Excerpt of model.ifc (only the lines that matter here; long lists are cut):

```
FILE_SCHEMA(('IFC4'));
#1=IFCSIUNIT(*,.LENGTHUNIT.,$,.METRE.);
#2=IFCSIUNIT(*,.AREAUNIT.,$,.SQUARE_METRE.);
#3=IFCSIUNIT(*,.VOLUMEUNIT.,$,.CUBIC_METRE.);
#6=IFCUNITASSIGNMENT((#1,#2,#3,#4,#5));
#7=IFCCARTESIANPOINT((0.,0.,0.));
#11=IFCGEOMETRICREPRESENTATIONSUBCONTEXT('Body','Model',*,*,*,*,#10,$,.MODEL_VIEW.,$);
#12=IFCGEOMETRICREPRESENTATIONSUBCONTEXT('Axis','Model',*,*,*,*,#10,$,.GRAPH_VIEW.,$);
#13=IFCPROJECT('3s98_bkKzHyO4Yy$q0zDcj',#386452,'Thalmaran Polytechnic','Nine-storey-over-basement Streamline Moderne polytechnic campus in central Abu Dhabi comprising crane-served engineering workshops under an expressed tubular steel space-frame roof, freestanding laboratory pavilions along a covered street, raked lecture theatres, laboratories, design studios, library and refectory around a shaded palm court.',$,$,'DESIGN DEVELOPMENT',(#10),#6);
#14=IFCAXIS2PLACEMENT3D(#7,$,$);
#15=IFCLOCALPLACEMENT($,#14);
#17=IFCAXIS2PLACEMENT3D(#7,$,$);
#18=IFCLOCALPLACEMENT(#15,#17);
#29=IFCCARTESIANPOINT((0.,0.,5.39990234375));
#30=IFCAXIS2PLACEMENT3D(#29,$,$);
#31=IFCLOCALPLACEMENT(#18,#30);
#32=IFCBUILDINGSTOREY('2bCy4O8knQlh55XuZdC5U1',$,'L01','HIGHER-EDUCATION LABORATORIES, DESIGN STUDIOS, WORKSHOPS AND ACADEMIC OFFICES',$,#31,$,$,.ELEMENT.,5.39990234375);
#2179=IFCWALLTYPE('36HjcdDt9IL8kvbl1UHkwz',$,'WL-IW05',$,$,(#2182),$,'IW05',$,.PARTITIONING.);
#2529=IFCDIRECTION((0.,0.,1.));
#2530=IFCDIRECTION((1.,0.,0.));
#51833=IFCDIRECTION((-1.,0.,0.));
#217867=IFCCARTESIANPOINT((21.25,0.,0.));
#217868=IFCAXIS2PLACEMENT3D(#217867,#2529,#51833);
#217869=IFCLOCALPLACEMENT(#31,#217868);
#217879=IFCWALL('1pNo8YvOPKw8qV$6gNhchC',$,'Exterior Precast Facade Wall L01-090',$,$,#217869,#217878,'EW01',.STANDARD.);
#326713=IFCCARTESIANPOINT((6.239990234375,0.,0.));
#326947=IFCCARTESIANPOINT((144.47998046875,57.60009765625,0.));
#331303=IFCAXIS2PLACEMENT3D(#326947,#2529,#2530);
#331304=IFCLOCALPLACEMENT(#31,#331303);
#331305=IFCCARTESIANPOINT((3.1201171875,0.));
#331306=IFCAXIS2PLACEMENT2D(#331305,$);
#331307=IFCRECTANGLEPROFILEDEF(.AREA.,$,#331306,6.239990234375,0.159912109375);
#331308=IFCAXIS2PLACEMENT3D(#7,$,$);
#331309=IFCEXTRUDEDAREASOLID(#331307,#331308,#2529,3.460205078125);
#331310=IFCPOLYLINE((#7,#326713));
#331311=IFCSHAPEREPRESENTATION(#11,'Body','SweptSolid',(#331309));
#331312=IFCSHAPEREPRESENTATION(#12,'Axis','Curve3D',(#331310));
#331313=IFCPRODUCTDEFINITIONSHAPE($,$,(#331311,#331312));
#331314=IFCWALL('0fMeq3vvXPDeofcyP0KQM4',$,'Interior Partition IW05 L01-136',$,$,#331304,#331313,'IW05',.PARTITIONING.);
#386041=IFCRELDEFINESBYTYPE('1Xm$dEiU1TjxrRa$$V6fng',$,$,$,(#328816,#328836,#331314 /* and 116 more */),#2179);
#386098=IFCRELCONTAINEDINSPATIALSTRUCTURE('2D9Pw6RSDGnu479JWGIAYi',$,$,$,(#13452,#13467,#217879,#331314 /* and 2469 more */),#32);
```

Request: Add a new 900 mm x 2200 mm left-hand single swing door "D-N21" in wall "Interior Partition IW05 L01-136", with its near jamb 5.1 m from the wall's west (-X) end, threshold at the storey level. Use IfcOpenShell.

```python
import numpy as np
import ifcopenshell
import ifcopenshell.api.feature
import ifcopenshell.api.geometry
import ifcopenshell.api.root
import ifcopenshell.api.spatial
import ifcopenshell.geom
import ifcopenshell.util.element
import ifcopenshell.util.placement
import ifcopenshell.util.representation
import ifcopenshell.util.shape
import ifcopenshell.util.unit

model = ifcopenshell.open("model.ifc")
unit_scale = ifcopenshell.util.unit.calculate_unit_scale(model)
settings = ifcopenshell.geom.settings()


def volume(element):
    """Net volume in cubic metres, openings subtracted."""
    shape = ifcopenshell.geom.create_shape(settings, element)
    return ifcopenshell.util.shape.get_volume(shape.geometry)


wall = model.by_guid("0fMeq3vvXPDeofcyP0KQM4")
storey = ifcopenshell.util.element.get_container(wall, ifc_class="IfcBuildingStorey")
context = ifcopenshell.util.representation.get_context(model, "Model", "Body", "MODEL_VIEW")
before = volume(wall)

width, height, from_end, sill = 0.9, 2.2, 5.1, 0.0  # metres

# The wall runs along its own X axis, and the end named is its -X end.
wall_shape = ifcopenshell.geom.create_shape(settings, wall)
x, y, z = ifcopenshell.util.shape.get_vertices(wall_shape.geometry).T
start = x.min() + from_end
face, thickness = float(y.min()), float(y.max() - y.min())
wall_matrix = ifcopenshell.util.placement.get_local_placement(wall.ObjectPlacement)
level = ifcopenshell.util.placement.get_local_placement(storey.ObjectPlacement)[2, 3]


def in_wall(x, y):
    """Placement at x, y metres in the wall's axes, at sill height."""
    matrix = wall_matrix.copy()
    matrix[:, 3] = wall_matrix @ np.array([x / unit_scale, y / unit_scale, 0.0, 1.0])
    matrix[2, 3] = level + sill / unit_scale
    return matrix


# Opening: a box that overshoots both wall faces by 50 mm.
opening = ifcopenshell.api.root.create_entity(model, ifc_class="IfcOpeningElement", predefined_type="OPENING")
box = ifcopenshell.api.geometry.add_wall_representation(
    model, context=context, length=width, height=height, thickness=thickness + 0.1
)
ifcopenshell.api.geometry.assign_representation(model, product=opening, representation=box)
ifcopenshell.api.geometry.edit_object_placement(model, product=opening, matrix=in_wall(start, face - 0.05), is_si=False)
ifcopenshell.api.feature.add_feature(model, feature=opening, element=wall)

door = ifcopenshell.api.root.create_entity(model, ifc_class="IfcDoor", name="D-N21", predefined_type="DOOR")
door.OverallWidth, door.OverallHeight = width / unit_scale, height / unit_scale
door.OperationType = "SINGLE_SWING_LEFT"
body = ifcopenshell.api.geometry.add_door_representation(
    model,
    context=context,
    overall_width=door.OverallWidth,
    overall_height=door.OverallHeight,
    operation_type="SINGLE_SWING_LEFT",
    lining_properties={"LiningDepth": thickness / unit_scale, "ThresholdDepth": thickness / unit_scale},
)
ifcopenshell.api.geometry.assign_representation(model, product=door, representation=body)
ifcopenshell.api.spatial.assign_container(model, products=[door], relating_structure=storey)
ifcopenshell.api.feature.add_filling(model, opening=opening, element=door)

# The lining spans the wall, so the door starts at the wall face.
ifcopenshell.api.geometry.edit_object_placement(model, product=door, matrix=in_wall(start, face), is_si=False)

after = volume(wall)

print(f"wall volume {before:.3f} -> {after:.3f} m3")

model.write("model-out.ifc")
```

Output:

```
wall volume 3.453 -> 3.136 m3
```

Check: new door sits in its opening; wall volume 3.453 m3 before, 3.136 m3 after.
